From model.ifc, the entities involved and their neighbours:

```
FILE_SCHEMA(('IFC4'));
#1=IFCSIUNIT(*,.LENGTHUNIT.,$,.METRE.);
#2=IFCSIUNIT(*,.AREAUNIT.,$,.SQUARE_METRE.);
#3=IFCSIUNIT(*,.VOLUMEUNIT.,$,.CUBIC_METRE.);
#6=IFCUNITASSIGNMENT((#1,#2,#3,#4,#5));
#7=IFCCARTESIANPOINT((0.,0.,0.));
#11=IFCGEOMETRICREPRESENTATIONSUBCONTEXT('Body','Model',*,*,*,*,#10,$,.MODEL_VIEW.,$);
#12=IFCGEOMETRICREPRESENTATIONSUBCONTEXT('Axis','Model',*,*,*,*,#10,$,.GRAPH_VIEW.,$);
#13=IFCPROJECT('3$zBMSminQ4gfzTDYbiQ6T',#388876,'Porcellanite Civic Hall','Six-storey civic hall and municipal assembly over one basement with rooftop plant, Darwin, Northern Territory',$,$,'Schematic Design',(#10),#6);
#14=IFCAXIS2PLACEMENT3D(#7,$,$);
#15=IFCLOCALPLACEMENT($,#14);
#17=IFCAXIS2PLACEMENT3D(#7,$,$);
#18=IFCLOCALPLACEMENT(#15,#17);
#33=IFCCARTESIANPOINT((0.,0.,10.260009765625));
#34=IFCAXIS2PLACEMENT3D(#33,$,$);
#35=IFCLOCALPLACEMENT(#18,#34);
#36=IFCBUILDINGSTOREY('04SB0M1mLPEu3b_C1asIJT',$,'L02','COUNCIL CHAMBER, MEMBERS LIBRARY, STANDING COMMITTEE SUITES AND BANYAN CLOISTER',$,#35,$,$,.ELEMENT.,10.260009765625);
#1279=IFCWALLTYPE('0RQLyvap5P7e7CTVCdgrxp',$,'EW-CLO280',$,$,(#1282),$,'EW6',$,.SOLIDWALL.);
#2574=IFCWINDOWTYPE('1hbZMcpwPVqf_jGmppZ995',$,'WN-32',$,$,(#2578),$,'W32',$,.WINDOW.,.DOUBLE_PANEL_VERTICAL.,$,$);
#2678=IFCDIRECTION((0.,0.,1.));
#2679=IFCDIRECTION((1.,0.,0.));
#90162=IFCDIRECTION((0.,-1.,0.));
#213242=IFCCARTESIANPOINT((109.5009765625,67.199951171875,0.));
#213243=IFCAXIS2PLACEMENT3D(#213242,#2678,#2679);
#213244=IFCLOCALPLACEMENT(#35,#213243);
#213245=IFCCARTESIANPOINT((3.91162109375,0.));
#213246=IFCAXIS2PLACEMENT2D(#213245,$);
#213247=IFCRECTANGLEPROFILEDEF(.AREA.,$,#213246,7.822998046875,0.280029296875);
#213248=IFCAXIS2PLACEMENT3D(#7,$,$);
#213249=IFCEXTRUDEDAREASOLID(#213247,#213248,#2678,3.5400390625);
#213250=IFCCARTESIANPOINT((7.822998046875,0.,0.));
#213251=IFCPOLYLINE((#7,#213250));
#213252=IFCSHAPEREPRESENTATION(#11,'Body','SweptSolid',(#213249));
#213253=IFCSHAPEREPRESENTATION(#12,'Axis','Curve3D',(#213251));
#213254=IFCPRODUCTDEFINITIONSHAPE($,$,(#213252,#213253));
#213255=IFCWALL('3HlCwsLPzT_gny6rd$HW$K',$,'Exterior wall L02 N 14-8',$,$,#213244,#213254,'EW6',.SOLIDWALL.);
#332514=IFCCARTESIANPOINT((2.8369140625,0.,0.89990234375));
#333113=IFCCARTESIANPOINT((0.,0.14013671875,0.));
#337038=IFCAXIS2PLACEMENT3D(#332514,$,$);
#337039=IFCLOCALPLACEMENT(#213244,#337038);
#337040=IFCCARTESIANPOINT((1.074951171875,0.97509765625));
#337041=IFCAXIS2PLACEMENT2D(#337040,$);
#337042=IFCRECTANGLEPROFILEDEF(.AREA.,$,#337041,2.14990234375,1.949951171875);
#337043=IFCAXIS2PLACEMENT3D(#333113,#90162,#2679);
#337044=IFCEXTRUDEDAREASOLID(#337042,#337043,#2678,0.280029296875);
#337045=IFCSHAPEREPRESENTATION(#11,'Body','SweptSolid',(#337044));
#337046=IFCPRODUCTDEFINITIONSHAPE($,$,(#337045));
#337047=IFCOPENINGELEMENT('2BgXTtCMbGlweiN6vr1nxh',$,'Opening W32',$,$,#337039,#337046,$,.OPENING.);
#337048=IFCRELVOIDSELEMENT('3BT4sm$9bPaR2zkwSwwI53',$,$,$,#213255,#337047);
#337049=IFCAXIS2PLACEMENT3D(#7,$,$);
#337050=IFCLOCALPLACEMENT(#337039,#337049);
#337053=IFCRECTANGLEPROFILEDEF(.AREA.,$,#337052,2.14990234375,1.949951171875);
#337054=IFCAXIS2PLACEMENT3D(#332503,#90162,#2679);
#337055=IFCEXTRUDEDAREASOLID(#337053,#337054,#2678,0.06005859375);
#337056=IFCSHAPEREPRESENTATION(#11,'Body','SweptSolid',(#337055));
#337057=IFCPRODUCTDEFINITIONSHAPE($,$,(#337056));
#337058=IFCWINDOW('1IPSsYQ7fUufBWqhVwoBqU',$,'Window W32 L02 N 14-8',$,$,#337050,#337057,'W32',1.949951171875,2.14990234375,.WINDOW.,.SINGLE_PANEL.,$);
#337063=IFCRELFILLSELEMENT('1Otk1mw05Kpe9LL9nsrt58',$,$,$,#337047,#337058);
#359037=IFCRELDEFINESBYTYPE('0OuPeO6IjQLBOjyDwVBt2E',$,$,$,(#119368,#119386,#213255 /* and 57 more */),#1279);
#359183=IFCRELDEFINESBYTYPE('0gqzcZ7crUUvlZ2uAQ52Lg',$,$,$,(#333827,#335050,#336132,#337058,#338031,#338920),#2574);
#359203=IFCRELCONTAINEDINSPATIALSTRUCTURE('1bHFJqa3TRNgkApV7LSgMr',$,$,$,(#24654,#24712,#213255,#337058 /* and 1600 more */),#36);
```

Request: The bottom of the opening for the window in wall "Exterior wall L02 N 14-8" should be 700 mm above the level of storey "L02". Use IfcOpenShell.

```python
import numpy as np
import ifcopenshell
import ifcopenshell.api.geometry
import ifcopenshell.geom
import ifcopenshell.util.element
import ifcopenshell.util.placement
import ifcopenshell.util.shape
import ifcopenshell.util.unit

model = ifcopenshell.open("model.ifc")
unit_scale = ifcopenshell.util.unit.calculate_unit_scale(model)

window = model.by_guid("1IPSsYQ7fUufBWqhVwoBqU")
opening = window.FillsVoids[0].RelatingOpeningElement
storey = ifcopenshell.util.element.get_container(window, ifc_class="IfcBuildingStorey")
level = ifcopenshell.util.placement.get_local_placement(storey.ObjectPlacement)[2, 3]

# The opening's origin need not be at the sill, so measure its lowest point.
shape = ifcopenshell.geom.create_shape(ifcopenshell.geom.settings(), opening)
bottom = ifcopenshell.util.shape.get_shape_bottom_elevation(shape, shape.geometry) / unit_scale
dz = level + 0.7 - bottom

shift = np.array([0.0, 0.0, dz])
# The window is placed relative to its opening, so it follows when the opening moves.
matrix = ifcopenshell.util.placement.get_local_placement(opening.ObjectPlacement)
matrix[:3, 3] += shift
ifcopenshell.api.geometry.edit_object_placement(
    model, product=opening, matrix=matrix, is_si=False, should_transform_children=True
)

print(f"moved by {dz * unit_scale:+.3f} m")

model.write("model_updated.ifc")
```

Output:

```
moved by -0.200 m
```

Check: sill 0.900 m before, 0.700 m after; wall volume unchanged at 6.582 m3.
